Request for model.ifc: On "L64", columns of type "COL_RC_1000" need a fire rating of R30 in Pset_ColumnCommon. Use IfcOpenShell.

First a look at what the model holds.

```python
import ifcopenshell
import ifcopenshell.util.element

model = ifcopenshell.open("model.ifc")
print(model.schema)
storey = next(s for s in model.by_type("IfcBuildingStorey") if s.Name == "L64")
columns = [e for e in ifcopenshell.util.element.get_decomposition(storey) if e.is_a("IfcColumn")]
seen = {}
for e in columns:
    element_type = ifcopenshell.util.element.get_type(e)
    key = (element_type.Name if element_type != e and element_type else None, ifcopenshell.util.element.get_pset(e, "Pset_ColumnCommon", "FireRating"))
    seen[key] = seen.get(key, 0) + 1
for (name, value), count in sorted(seen.items(), key=str):
    print(count, "x", name, "|", value)
```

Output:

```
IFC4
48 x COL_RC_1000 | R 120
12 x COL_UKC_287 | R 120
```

```python
import ifcopenshell
import ifcopenshell.api.pset
import ifcopenshell.util.element

model = ifcopenshell.open("model.ifc")

storey = next(s for s in model.by_type("IfcBuildingStorey") if s.Name == "L64")
columns = [e for e in ifcopenshell.util.element.get_decomposition(storey) if e.is_a("IfcColumn")]

count = 0
for e in columns:
    element_type = ifcopenshell.util.element.get_type(e)
    if element_type in (None, e) or element_type.Name != "COL_RC_1000":
        continue
    found = ifcopenshell.util.element.get_pset(e, "Pset_ColumnCommon", should_inherit=False)
    if found:
        pset = model.by_id(found["id"])
        if len(ifcopenshell.util.element.get_elements_by_pset(pset)) > 1:
            pset = ifcopenshell.api.pset.unshare_pset(model, products=[e], pset=pset)[0]
    else:
        pset = ifcopenshell.api.pset.add_pset(model, product=e, name="Pset_ColumnCommon")
    ifcopenshell.api.pset.edit_pset(model, pset=pset, properties={"FireRating": "R30"})
    count += 1

print(count, "columns updated")

model.write("model_v2.ifc")
```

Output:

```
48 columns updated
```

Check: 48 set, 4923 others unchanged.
